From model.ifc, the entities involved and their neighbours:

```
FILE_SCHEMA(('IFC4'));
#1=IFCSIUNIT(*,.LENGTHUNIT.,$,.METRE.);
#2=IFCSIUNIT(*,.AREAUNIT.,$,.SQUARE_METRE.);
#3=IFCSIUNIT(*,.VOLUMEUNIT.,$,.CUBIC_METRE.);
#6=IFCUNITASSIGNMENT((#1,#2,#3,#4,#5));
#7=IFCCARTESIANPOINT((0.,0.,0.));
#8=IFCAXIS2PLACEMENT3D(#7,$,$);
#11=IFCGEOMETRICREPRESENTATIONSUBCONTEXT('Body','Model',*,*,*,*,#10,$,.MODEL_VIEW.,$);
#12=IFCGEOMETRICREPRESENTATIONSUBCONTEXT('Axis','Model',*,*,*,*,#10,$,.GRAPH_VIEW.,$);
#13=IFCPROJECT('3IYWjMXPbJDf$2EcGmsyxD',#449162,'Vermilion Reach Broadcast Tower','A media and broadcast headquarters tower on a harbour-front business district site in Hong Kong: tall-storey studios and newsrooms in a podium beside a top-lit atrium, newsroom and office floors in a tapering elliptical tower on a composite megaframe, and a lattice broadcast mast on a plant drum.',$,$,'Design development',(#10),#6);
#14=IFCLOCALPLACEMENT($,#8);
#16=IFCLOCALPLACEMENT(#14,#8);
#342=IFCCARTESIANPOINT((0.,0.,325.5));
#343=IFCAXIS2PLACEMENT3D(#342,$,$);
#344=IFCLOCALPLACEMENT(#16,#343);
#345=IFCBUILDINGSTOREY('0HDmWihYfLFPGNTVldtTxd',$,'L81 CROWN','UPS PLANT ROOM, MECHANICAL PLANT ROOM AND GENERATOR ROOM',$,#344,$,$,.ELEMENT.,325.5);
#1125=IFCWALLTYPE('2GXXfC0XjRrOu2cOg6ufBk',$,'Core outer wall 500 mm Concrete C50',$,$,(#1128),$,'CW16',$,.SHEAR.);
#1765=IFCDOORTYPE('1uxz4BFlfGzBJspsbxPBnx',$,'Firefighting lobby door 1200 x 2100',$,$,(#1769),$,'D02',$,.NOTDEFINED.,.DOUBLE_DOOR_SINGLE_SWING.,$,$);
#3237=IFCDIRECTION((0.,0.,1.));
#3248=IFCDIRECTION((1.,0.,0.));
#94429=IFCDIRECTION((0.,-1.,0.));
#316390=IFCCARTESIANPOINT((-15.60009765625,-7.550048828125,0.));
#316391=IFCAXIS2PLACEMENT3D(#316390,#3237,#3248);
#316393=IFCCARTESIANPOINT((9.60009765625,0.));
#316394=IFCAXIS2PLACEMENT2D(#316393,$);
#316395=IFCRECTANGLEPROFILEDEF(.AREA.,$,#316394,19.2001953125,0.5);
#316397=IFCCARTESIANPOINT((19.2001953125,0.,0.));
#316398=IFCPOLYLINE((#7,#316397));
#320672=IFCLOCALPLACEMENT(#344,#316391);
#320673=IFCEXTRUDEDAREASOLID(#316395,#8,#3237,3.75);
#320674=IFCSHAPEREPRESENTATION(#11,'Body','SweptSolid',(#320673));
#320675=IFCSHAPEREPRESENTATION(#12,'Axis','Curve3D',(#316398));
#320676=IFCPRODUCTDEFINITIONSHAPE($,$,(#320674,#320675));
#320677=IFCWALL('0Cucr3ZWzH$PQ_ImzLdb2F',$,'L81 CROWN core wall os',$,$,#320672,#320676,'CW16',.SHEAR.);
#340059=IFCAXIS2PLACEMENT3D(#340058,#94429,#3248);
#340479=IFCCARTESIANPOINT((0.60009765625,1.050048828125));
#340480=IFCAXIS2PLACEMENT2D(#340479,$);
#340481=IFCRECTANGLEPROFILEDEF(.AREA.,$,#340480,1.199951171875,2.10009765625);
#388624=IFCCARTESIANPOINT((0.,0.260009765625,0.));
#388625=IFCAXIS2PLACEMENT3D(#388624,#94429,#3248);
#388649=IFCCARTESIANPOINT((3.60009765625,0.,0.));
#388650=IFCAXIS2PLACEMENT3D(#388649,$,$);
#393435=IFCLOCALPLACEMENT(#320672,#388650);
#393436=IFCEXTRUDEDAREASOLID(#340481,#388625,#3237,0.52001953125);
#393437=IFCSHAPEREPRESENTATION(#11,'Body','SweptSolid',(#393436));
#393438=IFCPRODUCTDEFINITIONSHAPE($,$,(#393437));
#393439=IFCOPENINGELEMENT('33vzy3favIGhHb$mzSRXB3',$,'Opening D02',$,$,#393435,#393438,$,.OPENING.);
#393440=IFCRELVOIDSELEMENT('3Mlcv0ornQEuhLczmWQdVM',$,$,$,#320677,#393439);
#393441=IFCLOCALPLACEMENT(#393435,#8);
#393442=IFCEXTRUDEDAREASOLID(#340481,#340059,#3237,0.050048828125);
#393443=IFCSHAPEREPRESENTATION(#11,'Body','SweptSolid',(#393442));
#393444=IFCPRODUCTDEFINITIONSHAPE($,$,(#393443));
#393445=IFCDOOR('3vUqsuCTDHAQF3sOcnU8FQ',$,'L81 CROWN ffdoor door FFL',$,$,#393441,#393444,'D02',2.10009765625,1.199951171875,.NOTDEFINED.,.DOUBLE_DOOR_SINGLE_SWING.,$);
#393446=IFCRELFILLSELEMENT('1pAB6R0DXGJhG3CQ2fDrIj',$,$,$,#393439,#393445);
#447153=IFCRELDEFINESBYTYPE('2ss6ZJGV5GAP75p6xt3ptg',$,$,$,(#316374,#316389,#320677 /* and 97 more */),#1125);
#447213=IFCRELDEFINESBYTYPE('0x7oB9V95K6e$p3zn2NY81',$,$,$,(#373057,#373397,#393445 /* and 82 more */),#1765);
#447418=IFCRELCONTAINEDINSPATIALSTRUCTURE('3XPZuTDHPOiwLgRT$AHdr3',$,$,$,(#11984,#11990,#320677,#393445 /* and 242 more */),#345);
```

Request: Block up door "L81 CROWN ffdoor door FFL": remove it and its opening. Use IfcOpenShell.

```python
import ifcopenshell
import ifcopenshell.api.feature
import ifcopenshell.api.root
import ifcopenshell.geom
import ifcopenshell.util.shape

model = ifcopenshell.open("model.ifc")
settings = ifcopenshell.geom.settings()


def volume(element):
    """Net volume in cubic metres, openings subtracted."""
    shape = ifcopenshell.geom.create_shape(settings, element)
    return ifcopenshell.util.shape.get_volume(shape.geometry)


door = model.by_id(393445)
opening = door.FillsVoids[0].RelatingOpeningElement
wall = opening.VoidsElements[0].RelatingBuildingElement
before = volume(wall)

ifcopenshell.api.root.remove_product(model, product=door)
ifcopenshell.api.feature.remove_feature(model, feature=opening)

after = volume(wall)

print(f"wall volume {before:.3f} -> {after:.3f} m3")

model.write("model-out.ifc")
```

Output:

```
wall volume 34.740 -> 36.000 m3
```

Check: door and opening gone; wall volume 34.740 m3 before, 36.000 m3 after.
